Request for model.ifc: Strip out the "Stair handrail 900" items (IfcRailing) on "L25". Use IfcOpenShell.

First a look at what the model holds.

```python
import ifcopenshell
import ifcopenshell.util.element

model = ifcopenshell.open("model.ifc")
print(model.schema)
storey = next(s for s in model.by_type("IfcBuildingStorey") if s.Name == "L25")
railings = [e for e in ifcopenshell.util.element.get_decomposition(storey) if e.is_a("IfcRailing")]
seen = {}
for e in railings:
    element_type = ifcopenshell.util.element.get_type(e)
    name = element_type.Name if element_type not in (None, e) else None
    seen[name] = seen.get(name, 0) + 1
for name, count in sorted(seen.items(), key=str):
    print(count, "x", name)
```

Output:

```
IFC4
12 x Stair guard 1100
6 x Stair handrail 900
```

```python
import ifcopenshell
import ifcopenshell.api.root
import ifcopenshell.util.element

model = ifcopenshell.open("model.ifc")

storey = next(s for s in model.by_type("IfcBuildingStorey") if s.Name == "L25")
railings = [e for e in ifcopenshell.util.element.get_decomposition(storey) if e.is_a("IfcRailing")]
targets = [e for e in railings if (t := ifcopenshell.util.element.get_type(e)) not in (None, e) and t.Name == "Stair handrail 900"]

for e in targets:
    ifcopenshell.api.root.remove_product(model, product=e)
print(len(targets), "removed")

model.write("model_v2.ifc")
```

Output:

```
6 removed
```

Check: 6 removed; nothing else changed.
